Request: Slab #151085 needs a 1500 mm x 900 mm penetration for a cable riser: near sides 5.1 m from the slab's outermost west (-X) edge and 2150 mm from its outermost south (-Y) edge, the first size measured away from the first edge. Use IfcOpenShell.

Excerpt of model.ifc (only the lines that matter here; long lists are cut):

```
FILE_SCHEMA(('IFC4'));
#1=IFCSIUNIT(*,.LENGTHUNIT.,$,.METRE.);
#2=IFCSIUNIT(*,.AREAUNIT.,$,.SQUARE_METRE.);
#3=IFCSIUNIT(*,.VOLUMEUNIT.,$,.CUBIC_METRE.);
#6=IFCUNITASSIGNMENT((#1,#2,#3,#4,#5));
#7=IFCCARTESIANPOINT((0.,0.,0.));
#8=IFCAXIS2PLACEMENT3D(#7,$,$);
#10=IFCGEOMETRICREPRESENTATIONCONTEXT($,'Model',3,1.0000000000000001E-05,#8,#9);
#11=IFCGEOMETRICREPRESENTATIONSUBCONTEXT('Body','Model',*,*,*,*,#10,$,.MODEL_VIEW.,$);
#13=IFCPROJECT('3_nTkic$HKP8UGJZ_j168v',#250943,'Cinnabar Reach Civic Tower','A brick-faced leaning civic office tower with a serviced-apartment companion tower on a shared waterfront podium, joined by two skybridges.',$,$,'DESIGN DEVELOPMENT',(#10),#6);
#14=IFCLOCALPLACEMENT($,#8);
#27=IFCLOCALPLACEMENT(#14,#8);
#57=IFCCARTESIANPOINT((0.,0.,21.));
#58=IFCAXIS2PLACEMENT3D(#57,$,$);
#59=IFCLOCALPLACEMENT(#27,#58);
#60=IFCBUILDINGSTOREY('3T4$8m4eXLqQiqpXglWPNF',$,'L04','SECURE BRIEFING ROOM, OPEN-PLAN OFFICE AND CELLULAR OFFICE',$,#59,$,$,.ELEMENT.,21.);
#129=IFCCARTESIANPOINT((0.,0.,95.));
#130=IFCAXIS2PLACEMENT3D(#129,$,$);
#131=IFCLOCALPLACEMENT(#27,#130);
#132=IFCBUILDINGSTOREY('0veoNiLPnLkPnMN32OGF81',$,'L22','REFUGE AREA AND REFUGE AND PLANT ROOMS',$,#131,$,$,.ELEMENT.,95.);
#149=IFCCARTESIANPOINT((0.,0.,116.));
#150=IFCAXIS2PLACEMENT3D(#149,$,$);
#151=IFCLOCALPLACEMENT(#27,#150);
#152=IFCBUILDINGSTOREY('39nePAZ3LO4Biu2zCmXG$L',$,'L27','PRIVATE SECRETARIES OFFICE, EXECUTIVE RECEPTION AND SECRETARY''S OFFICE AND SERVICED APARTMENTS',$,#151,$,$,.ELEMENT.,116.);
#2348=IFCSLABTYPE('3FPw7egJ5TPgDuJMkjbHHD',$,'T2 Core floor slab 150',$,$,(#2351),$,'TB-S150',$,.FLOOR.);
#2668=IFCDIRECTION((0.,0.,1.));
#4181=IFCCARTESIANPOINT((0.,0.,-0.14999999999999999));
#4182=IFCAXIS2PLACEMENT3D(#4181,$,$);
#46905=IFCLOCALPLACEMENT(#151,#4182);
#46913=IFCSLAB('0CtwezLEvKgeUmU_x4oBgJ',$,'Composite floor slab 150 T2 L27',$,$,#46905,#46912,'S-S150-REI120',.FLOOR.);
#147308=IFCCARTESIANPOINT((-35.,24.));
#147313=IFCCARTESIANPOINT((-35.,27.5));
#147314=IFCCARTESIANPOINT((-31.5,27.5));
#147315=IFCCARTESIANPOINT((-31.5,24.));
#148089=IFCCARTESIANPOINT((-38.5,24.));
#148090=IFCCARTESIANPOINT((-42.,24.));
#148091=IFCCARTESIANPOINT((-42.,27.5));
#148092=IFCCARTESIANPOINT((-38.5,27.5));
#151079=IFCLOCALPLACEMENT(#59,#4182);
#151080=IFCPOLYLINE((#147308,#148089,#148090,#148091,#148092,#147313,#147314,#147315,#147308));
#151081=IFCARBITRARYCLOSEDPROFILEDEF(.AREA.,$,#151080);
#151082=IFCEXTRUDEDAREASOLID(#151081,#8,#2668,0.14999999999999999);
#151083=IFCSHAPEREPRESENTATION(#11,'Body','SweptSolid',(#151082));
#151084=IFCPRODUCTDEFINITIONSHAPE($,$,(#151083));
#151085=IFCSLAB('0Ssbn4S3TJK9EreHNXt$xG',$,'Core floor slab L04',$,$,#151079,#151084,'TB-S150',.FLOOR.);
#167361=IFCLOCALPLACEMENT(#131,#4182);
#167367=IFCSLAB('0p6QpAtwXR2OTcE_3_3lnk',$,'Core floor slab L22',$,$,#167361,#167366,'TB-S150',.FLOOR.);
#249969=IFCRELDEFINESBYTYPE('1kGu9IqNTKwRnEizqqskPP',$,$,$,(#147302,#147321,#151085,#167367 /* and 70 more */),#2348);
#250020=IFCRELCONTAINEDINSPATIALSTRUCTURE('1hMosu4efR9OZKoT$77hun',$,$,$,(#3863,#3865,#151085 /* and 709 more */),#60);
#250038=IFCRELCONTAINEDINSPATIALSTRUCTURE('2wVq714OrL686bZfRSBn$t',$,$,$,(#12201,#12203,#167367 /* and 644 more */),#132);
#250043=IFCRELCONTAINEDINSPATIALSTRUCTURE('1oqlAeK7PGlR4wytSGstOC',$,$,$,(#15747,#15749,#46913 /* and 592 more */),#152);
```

```python
import numpy as np
import ifcopenshell
import ifcopenshell.api.feature
import ifcopenshell.api.geometry
import ifcopenshell.api.root
import ifcopenshell.geom
import ifcopenshell.util.placement
import ifcopenshell.util.representation
import ifcopenshell.util.shape
import ifcopenshell.util.unit

model = ifcopenshell.open("model.ifc")
unit_scale = ifcopenshell.util.unit.calculate_unit_scale(model)
settings = ifcopenshell.geom.settings()


def volume(element):
    """Net volume in cubic metres, openings subtracted."""
    shape = ifcopenshell.geom.create_shape(settings, element)
    return ifcopenshell.util.shape.get_volume(shape.geometry)


slab = model.by_id(151085)
before = volume(slab)

# Extent in the slab's own axes, in metres. The edges named are its -X and -Y sides.
slab_shape = ifcopenshell.geom.create_shape(settings, slab)
vertices = ifcopenshell.util.shape.get_vertices(slab_shape.geometry)
x_min, y_min, bottom = vertices.min(axis=0)
top = vertices[:, 2].max()

opening = ifcopenshell.api.root.create_entity(model, ifc_class="IfcOpeningElement", name="Cable riser opening", predefined_type="OPENING")
context = ifcopenshell.util.representation.get_context(model, "Model", "Body", "MODEL_VIEW")
width, depth = 1.5, 0.9
outline = [(0.0, 0.0), (width, 0.0), (width, depth), (0.0, depth), (0.0, 0.0)]
# Overshoot both faces by 50 mm so the cut is clean.
shape = ifcopenshell.api.geometry.add_slab_representation(
    model, context=context, depth=top - bottom + 0.1, polyline=outline
)
ifcopenshell.api.geometry.assign_representation(model, product=opening, representation=shape)

matrix = ifcopenshell.util.placement.get_local_placement(slab.ObjectPlacement)
matrix[:, 3] = matrix @ np.append(np.array([x_min + 5.1, y_min + 2.15, bottom - 0.05]) / unit_scale, 1.0)
ifcopenshell.api.geometry.edit_object_placement(model, product=opening, matrix=matrix, is_si=False)
ifcopenshell.api.feature.add_feature(model, feature=opening, element=slab)

after = volume(slab)

print(f"slab volume {before:.3f} -> {after:.3f} m3")

model.write("model-out.ifc")
```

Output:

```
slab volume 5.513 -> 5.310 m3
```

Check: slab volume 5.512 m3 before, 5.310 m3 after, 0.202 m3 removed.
